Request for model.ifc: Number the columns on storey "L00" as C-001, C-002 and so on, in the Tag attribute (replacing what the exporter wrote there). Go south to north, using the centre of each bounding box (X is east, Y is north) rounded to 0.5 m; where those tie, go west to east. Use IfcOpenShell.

First a look at what the model holds.

```python
import ifcopenshell
import ifcopenshell.util.element
import ifcopenshell.util.placement

model = ifcopenshell.open("model.ifc")
print(model.schema)
storey = next(s for s in model.by_type("IfcBuildingStorey") if s.Name == "L00")
columns = [e for e in ifcopenshell.util.element.get_decomposition(storey) if e.is_a("IfcColumn")]
for e in sorted(columns, key=lambda e: e.id()):
    origin = ifcopenshell.util.placement.get_local_placement(e.ObjectPlacement)[:3, 3]
    print(e.id(), e.Tag, e.Name, origin.round(2) + 0.0, sep=" | ")
```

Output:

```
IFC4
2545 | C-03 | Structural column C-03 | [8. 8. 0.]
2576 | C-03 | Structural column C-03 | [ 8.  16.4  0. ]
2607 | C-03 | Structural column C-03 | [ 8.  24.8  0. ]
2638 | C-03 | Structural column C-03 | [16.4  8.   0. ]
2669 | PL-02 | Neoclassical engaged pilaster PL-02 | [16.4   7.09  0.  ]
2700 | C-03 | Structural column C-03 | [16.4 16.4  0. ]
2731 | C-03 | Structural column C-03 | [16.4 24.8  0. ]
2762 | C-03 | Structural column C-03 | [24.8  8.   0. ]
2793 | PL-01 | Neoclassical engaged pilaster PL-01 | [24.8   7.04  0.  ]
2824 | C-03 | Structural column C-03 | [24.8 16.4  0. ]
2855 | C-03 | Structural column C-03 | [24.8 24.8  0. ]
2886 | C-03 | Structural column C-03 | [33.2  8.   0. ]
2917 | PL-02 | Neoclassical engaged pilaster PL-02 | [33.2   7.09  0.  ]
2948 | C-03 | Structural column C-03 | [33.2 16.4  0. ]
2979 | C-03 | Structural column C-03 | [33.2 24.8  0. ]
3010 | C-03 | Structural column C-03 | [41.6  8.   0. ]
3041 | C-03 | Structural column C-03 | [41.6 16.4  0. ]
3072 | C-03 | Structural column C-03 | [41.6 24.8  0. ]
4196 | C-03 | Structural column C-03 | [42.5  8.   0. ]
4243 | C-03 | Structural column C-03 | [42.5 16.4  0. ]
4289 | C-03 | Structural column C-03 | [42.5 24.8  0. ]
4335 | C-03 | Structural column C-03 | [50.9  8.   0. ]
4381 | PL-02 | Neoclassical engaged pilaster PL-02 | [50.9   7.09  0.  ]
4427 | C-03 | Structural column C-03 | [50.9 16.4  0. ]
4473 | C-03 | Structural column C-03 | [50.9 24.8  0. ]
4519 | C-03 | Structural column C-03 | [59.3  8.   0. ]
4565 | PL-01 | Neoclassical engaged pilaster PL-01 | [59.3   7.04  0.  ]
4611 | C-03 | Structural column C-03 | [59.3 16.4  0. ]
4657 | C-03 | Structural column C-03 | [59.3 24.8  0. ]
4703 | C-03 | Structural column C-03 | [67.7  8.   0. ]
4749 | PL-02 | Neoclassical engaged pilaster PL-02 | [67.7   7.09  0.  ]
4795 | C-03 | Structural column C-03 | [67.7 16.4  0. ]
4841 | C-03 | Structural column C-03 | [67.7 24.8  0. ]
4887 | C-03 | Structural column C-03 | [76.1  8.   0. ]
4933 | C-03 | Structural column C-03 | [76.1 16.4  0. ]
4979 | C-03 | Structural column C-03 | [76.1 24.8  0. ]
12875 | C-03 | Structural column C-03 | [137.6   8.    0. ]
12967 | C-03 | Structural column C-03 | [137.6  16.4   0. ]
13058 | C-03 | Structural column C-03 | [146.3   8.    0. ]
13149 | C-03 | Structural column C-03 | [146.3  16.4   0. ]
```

```python
import ifcopenshell
import ifcopenshell.geom
import ifcopenshell.util.element
import ifcopenshell.util.shape

model = ifcopenshell.open("model.ifc")
settings = ifcopenshell.geom.settings()
settings.set("use-world-coords", True)


def centre(element):
    shape = ifcopenshell.geom.create_shape(settings, element)
    return ifcopenshell.util.shape.get_bbox_centroid(shape.geometry)


storey = next(s for s in model.by_type("IfcBuildingStorey") if s.Name == "L00")
columns = [e for e in ifcopenshell.util.element.get_decomposition(storey) if e.is_a("IfcColumn")]

# Insertion points can sit at a corner or the storey origin, so sort by the geometry (in metres).
centres = {e: centre(e) for e in columns}
columns.sort(key=lambda e: (round(centres[e][1] / 0.5), centres[e][0]))

for i, e in enumerate(columns, start=1):
    number = f"C-0{i:02d}"
    e.Tag = number
    print(e.id(), number)

model.write("model_edited.ifc")
```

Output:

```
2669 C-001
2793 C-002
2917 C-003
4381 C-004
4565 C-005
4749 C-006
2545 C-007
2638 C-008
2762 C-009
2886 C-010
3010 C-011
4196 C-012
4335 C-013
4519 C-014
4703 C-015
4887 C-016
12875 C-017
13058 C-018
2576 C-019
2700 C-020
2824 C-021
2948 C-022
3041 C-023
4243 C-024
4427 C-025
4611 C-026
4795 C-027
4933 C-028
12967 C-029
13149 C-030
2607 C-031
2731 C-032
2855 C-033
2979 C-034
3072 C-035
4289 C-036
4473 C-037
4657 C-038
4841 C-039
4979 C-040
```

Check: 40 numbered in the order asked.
